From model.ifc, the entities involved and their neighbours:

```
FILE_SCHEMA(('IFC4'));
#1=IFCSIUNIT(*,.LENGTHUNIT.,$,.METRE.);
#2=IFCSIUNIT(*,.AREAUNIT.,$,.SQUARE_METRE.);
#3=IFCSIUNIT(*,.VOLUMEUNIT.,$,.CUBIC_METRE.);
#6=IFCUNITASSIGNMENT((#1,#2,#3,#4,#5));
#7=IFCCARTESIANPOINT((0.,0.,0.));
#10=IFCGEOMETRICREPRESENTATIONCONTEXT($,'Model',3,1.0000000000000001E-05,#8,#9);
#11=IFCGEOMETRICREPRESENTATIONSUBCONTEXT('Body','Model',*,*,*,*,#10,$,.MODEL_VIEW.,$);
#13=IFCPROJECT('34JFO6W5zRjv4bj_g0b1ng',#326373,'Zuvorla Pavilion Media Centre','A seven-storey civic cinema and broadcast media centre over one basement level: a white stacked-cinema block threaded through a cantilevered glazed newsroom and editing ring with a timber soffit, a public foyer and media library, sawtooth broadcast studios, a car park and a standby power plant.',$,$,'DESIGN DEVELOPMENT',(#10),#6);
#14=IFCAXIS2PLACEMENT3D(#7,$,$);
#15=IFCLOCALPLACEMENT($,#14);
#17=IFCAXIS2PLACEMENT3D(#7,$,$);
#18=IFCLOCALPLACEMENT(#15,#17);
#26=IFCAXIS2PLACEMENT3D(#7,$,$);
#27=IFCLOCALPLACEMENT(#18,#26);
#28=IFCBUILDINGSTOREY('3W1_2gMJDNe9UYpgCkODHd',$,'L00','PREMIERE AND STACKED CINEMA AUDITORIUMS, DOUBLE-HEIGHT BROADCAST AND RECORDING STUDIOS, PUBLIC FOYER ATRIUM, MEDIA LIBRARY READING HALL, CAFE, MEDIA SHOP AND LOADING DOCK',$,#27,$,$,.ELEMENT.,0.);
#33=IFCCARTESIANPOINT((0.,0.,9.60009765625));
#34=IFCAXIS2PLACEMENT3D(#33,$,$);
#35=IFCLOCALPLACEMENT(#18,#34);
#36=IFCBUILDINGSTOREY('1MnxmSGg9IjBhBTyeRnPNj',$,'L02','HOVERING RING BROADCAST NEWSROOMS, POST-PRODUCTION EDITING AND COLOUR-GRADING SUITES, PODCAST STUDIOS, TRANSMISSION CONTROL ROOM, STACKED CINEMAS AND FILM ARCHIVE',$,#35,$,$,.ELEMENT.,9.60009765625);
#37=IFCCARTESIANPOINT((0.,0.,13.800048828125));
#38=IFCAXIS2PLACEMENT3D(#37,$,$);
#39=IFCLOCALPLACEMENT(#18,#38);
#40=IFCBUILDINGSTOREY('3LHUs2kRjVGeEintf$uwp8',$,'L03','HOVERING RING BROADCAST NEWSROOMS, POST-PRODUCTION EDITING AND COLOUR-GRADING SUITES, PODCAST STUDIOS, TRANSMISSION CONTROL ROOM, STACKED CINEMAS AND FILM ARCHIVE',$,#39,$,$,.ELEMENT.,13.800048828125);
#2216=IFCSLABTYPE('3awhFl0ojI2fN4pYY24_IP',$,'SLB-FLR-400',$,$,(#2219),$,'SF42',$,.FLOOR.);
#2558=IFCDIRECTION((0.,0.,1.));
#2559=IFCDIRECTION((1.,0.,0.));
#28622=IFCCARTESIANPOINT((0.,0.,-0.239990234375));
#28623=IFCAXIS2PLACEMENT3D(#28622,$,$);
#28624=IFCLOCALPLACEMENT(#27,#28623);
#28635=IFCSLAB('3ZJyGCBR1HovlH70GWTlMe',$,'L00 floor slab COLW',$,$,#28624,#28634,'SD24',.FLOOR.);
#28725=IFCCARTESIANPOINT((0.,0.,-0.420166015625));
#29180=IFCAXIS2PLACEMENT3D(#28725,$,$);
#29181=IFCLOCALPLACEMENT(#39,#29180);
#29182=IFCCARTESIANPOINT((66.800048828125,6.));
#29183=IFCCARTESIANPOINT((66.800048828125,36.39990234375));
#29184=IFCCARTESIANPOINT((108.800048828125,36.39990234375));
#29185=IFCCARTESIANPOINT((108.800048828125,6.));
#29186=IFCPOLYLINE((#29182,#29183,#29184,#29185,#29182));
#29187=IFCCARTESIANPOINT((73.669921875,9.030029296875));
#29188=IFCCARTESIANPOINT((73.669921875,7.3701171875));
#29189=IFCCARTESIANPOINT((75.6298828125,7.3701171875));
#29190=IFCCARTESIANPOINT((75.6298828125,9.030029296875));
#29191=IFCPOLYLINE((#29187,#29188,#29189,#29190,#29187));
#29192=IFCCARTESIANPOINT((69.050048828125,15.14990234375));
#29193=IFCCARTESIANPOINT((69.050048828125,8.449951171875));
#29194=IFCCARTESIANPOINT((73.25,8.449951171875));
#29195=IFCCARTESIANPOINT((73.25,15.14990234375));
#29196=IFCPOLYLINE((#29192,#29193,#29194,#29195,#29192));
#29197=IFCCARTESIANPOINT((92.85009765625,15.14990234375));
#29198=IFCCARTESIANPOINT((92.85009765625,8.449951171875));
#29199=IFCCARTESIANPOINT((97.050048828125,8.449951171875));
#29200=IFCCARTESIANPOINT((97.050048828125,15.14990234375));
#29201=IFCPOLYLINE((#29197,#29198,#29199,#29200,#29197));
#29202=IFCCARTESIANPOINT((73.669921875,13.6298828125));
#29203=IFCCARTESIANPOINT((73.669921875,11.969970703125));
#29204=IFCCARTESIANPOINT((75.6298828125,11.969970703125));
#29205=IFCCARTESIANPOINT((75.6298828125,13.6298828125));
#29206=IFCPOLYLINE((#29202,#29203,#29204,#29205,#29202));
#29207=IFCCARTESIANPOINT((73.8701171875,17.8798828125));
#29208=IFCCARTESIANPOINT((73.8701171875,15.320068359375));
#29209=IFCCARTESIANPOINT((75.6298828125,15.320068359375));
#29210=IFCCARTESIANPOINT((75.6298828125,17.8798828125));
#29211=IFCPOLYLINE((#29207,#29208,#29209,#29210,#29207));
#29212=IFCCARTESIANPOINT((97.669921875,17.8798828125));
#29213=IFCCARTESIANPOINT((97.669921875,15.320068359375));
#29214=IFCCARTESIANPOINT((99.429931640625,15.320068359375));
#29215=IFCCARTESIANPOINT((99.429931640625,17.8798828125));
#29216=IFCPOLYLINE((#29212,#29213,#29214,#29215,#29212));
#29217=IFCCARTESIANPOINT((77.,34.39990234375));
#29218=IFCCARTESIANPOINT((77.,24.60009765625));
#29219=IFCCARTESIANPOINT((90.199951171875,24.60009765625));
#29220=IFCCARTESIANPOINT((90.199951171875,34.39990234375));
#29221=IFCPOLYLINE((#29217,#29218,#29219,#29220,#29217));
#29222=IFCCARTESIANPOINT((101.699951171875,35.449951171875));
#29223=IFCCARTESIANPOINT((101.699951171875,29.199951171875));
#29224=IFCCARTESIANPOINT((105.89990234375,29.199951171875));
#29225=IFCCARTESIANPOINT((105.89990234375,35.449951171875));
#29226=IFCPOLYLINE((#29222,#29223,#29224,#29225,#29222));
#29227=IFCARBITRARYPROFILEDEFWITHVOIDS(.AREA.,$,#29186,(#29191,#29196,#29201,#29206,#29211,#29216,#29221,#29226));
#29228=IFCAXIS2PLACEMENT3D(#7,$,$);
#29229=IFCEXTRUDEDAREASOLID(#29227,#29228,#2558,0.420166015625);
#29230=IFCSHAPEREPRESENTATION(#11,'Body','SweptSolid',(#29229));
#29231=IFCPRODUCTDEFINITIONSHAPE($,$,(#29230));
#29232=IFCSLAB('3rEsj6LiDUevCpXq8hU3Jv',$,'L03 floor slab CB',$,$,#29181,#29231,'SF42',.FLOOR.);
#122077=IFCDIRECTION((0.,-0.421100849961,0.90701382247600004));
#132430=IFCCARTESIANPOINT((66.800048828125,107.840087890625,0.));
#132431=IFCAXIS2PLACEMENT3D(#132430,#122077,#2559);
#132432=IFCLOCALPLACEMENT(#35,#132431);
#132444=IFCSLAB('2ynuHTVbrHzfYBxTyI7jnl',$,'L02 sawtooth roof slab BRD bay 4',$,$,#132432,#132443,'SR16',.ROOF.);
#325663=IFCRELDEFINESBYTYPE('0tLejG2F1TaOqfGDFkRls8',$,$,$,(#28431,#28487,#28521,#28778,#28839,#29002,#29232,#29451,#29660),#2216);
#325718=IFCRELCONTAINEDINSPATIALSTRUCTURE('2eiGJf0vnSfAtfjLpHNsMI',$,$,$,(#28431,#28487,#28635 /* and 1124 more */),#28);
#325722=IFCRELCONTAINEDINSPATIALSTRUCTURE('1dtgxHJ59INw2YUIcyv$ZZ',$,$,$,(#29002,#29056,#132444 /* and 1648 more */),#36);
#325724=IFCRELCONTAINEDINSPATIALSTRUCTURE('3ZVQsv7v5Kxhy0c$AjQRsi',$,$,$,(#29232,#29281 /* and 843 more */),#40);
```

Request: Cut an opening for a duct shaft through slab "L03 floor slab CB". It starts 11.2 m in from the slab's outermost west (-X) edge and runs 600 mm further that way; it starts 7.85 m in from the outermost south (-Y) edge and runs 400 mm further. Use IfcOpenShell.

```python
import numpy as np
import ifcopenshell
import ifcopenshell.api.feature
import ifcopenshell.api.geometry
import ifcopenshell.api.root
import ifcopenshell.geom
import ifcopenshell.util.placement
import ifcopenshell.util.representation
import ifcopenshell.util.shape
import ifcopenshell.util.unit

model = ifcopenshell.open("model.ifc")
unit_scale = ifcopenshell.util.unit.calculate_unit_scale(model)
settings = ifcopenshell.geom.settings()


def volume(element):
    """Net volume in cubic metres, openings subtracted."""
    shape = ifcopenshell.geom.create_shape(settings, element)
    return ifcopenshell.util.shape.get_volume(shape.geometry)


slab = model.by_guid("3rEsj6LiDUevCpXq8hU3Jv")
before = volume(slab)

# Extent in the slab's own axes, in metres. The edges named are its -X and -Y sides.
slab_shape = ifcopenshell.geom.create_shape(settings, slab)
vertices = ifcopenshell.util.shape.get_vertices(slab_shape.geometry)
x_min, y_min, bottom = vertices.min(axis=0)
top = vertices[:, 2].max()

opening = ifcopenshell.api.root.create_entity(model, ifc_class="IfcOpeningElement", name="Duct shaft opening", predefined_type="OPENING")
context = ifcopenshell.util.representation.get_context(model, "Model", "Body", "MODEL_VIEW")
width, depth = 0.6, 0.4
outline = [(0.0, 0.0), (width, 0.0), (width, depth), (0.0, depth), (0.0, 0.0)]
# Overshoot both faces by 50 mm so the cut is clean.
shape = ifcopenshell.api.geometry.add_slab_representation(
    model, context=context, depth=top - bottom + 0.1, polyline=outline
)
ifcopenshell.api.geometry.assign_representation(model, product=opening, representation=shape)

matrix = ifcopenshell.util.placement.get_local_placement(slab.ObjectPlacement)
matrix[:, 3] = matrix @ np.append(np.array([x_min + 11.2, y_min + 7.85, bottom - 0.05]) / unit_scale, 1.0)
ifcopenshell.api.geometry.edit_object_placement(model, product=opening, matrix=matrix, is_si=False)
ifcopenshell.api.feature.add_feature(model, feature=opening, element=slab)

after = volume(slab)

print(f"slab volume {before:.3f} -> {after:.3f} m3")

model.write("model_edited.ifc")
```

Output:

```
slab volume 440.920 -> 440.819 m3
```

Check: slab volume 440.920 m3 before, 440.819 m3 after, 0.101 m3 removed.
